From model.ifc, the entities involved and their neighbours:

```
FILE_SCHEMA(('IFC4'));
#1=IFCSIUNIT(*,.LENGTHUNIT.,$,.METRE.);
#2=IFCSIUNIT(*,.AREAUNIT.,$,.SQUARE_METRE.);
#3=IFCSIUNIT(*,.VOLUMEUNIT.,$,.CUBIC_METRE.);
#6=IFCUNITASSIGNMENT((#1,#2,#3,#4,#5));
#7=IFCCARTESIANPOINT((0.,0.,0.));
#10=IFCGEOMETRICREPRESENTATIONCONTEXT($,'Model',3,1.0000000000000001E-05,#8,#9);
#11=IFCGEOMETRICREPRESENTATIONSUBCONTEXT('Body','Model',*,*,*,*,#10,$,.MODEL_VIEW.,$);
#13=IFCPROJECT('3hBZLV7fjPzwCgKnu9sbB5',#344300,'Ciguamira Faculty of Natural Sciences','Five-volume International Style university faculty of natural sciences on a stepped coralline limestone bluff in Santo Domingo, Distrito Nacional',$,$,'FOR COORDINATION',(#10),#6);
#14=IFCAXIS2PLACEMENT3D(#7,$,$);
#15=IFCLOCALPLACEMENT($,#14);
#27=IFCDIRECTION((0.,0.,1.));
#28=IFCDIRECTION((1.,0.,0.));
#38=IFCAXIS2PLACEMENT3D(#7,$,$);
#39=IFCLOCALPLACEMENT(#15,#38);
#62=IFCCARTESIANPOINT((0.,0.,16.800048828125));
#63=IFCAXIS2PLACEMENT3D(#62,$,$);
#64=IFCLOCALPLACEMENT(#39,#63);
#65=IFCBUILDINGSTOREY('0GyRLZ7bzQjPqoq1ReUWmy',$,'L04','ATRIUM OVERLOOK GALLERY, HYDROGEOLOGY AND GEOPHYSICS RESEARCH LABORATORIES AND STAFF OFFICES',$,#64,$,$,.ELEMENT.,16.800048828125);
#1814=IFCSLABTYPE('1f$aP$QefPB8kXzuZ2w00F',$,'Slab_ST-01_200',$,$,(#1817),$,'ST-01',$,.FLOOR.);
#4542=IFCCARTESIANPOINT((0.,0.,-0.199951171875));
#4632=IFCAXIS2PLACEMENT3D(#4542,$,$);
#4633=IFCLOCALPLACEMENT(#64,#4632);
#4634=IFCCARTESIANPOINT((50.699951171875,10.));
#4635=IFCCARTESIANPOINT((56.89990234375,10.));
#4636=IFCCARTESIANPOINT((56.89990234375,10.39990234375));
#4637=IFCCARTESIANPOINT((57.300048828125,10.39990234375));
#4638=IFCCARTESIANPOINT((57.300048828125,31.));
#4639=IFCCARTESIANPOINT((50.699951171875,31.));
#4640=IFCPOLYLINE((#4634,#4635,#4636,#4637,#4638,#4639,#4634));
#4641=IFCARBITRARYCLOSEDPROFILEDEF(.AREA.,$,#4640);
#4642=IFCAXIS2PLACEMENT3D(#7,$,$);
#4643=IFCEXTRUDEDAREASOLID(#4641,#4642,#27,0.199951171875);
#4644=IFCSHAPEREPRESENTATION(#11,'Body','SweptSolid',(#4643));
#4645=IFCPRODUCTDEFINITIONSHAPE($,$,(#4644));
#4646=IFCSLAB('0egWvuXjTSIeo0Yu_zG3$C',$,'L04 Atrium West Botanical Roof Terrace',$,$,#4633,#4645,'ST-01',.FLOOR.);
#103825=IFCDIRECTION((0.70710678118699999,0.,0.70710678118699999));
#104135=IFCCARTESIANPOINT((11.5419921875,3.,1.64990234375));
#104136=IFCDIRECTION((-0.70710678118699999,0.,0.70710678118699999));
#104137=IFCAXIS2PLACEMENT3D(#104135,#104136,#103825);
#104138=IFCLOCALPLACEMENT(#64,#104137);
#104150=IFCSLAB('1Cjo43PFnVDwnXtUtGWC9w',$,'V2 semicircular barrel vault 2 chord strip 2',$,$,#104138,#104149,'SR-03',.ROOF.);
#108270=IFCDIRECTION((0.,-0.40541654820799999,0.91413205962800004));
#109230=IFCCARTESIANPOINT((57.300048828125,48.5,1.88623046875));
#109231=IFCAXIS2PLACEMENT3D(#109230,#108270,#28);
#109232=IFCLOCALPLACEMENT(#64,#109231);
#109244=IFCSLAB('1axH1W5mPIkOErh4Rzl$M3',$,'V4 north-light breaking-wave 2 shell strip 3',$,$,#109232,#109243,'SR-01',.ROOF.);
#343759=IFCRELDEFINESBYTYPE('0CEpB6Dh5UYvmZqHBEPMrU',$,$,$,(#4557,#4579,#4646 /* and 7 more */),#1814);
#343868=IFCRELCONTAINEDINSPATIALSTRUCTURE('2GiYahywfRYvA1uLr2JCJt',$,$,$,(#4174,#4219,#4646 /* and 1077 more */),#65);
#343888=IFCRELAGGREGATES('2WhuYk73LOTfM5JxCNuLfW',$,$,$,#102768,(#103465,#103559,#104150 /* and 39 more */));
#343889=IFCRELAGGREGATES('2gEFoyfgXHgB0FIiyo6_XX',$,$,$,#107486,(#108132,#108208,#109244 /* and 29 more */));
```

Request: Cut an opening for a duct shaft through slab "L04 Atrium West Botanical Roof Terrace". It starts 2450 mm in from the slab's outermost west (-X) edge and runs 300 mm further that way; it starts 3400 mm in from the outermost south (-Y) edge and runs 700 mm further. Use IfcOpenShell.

```python
import numpy as np
import ifcopenshell
import ifcopenshell.api.feature
import ifcopenshell.api.geometry
import ifcopenshell.api.root
import ifcopenshell.geom
import ifcopenshell.util.placement
import ifcopenshell.util.representation
import ifcopenshell.util.shape
import ifcopenshell.util.unit

model = ifcopenshell.open("model.ifc")
unit_scale = ifcopenshell.util.unit.calculate_unit_scale(model)
settings = ifcopenshell.geom.settings()


def volume(element):
    """Net volume in cubic metres, openings subtracted."""
    shape = ifcopenshell.geom.create_shape(settings, element)
    return ifcopenshell.util.shape.get_volume(shape.geometry)


slab = model.by_guid("0egWvuXjTSIeo0Yu_zG3$C")
before = volume(slab)

# Extent in the slab's own axes, in metres. The edges named are its -X and -Y sides.
slab_shape = ifcopenshell.geom.create_shape(settings, slab)
vertices = ifcopenshell.util.shape.get_vertices(slab_shape.geometry)
x_min, y_min, bottom = vertices.min(axis=0)
top = vertices[:, 2].max()

opening = ifcopenshell.api.root.create_entity(model, ifc_class="IfcOpeningElement", name="Duct shaft opening", predefined_type="OPENING")
context = ifcopenshell.util.representation.get_context(model, "Model", "Body", "MODEL_VIEW")
width, depth = 0.3, 0.7
outline = [(0.0, 0.0), (width, 0.0), (width, depth), (0.0, depth), (0.0, 0.0)]
# Overshoot both faces by 50 mm so the cut is clean.
shape = ifcopenshell.api.geometry.add_slab_representation(
    model, context=context, depth=top - bottom + 0.1, polyline=outline
)
ifcopenshell.api.geometry.assign_representation(model, product=opening, representation=shape)

matrix = ifcopenshell.util.placement.get_local_placement(slab.ObjectPlacement)
matrix[:, 3] = matrix @ np.append(np.array([x_min + 2.45, y_min + 3.4, bottom - 0.05]) / unit_scale, 1.0)
ifcopenshell.api.geometry.edit_object_placement(model, product=opening, matrix=matrix, is_si=False)
ifcopenshell.api.feature.add_feature(model, feature=opening, element=slab)

after = volume(slab)

print(f"slab volume {before:.3f} -> {after:.3f} m3")

model.write("model_edited.ifc")
```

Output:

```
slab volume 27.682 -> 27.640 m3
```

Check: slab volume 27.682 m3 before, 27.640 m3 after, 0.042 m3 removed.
